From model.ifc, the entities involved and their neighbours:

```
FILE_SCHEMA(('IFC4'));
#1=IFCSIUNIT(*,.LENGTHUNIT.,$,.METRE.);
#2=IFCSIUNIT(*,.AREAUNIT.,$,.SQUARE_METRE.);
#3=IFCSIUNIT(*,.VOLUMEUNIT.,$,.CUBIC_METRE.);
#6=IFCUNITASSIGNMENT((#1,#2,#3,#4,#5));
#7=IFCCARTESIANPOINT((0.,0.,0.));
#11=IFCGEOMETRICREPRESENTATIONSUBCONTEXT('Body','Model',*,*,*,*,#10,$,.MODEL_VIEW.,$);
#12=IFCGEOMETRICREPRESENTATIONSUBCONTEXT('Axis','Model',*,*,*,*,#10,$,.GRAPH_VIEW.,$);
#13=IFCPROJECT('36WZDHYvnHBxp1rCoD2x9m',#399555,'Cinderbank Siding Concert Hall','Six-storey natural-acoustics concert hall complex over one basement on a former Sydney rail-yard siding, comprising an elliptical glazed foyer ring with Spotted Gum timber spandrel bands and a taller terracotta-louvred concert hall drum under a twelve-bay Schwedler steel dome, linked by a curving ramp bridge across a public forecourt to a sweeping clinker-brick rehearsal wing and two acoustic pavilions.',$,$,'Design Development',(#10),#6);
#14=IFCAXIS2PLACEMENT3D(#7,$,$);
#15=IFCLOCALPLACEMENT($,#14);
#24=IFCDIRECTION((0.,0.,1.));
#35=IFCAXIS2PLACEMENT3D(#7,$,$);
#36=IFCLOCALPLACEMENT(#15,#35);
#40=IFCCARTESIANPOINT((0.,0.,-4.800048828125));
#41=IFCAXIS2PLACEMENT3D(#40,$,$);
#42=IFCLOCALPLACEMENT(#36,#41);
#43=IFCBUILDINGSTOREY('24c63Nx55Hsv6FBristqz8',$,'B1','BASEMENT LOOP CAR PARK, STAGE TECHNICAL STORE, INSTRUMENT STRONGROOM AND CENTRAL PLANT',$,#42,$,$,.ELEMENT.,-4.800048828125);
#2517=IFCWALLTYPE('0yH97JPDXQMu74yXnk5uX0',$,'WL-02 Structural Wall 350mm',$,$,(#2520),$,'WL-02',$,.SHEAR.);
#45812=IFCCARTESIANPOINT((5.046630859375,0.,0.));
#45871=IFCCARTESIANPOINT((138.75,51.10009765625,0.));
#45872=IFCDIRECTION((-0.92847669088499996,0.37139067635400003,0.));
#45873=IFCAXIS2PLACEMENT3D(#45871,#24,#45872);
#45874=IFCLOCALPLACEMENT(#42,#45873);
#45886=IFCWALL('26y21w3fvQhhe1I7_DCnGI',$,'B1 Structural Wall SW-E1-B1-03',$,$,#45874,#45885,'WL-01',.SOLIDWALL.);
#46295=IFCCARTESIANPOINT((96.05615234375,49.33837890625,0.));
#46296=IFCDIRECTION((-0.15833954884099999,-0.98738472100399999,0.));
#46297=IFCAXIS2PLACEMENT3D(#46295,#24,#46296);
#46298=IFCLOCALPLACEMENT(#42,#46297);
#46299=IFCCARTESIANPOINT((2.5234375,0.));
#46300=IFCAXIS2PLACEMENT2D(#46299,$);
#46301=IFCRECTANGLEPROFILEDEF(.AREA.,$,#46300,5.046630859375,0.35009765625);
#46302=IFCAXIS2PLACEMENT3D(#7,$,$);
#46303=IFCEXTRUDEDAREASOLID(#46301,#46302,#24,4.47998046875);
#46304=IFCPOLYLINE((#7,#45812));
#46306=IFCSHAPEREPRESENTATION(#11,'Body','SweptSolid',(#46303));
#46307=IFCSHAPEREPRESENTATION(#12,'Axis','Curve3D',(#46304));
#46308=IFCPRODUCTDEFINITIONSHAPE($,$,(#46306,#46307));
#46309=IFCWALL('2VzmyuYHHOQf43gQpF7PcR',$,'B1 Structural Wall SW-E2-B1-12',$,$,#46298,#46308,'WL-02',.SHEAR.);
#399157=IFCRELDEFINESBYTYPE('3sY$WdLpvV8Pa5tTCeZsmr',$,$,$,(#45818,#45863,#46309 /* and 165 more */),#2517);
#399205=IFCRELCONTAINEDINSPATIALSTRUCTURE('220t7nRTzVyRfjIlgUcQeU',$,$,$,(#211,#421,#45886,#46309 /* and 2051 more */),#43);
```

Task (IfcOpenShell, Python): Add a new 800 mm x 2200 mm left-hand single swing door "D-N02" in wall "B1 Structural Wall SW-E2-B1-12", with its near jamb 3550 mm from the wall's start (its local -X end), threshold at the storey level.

```python
import numpy as np
import ifcopenshell
import ifcopenshell.api.feature
import ifcopenshell.api.geometry
import ifcopenshell.api.root
import ifcopenshell.api.spatial
import ifcopenshell.geom
import ifcopenshell.util.element
import ifcopenshell.util.placement
import ifcopenshell.util.representation
import ifcopenshell.util.shape
import ifcopenshell.util.unit

model = ifcopenshell.open("model.ifc")
unit_scale = ifcopenshell.util.unit.calculate_unit_scale(model)
settings = ifcopenshell.geom.settings()


def volume(element):
    """Net volume in cubic metres, openings subtracted."""
    shape = ifcopenshell.geom.create_shape(settings, element)
    return ifcopenshell.util.shape.get_volume(shape.geometry)


wall = model.by_guid("2VzmyuYHHOQf43gQpF7PcR")
storey = ifcopenshell.util.element.get_container(wall, ifc_class="IfcBuildingStorey")
context = ifcopenshell.util.representation.get_context(model, "Model", "Body", "MODEL_VIEW")
before = volume(wall)

width, height, from_end, sill = 0.8, 2.2, 3.55, 0.0  # metres

# The wall runs along its own X axis, and the end named is its -X end.
wall_shape = ifcopenshell.geom.create_shape(settings, wall)
x, y, z = ifcopenshell.util.shape.get_vertices(wall_shape.geometry).T
start = x.min() + from_end
face, thickness = float(y.min()), float(y.max() - y.min())
wall_matrix = ifcopenshell.util.placement.get_local_placement(wall.ObjectPlacement)
level = ifcopenshell.util.placement.get_local_placement(storey.ObjectPlacement)[2, 3]


def in_wall(x, y):
    """Placement at x, y metres in the wall's axes, at sill height."""
    matrix = wall_matrix.copy()
    matrix[:, 3] = wall_matrix @ np.array([x / unit_scale, y / unit_scale, 0.0, 1.0])
    matrix[2, 3] = level + sill / unit_scale
    return matrix


# Opening: a box that overshoots both wall faces by 50 mm.
opening = ifcopenshell.api.root.create_entity(model, ifc_class="IfcOpeningElement", predefined_type="OPENING")
box = ifcopenshell.api.geometry.add_wall_representation(
    model, context=context, length=width, height=height, thickness=thickness + 0.1
)
ifcopenshell.api.geometry.assign_representation(model, product=opening, representation=box)
ifcopenshell.api.geometry.edit_object_placement(model, product=opening, matrix=in_wall(start, face - 0.05), is_si=False)
ifcopenshell.api.feature.add_feature(model, feature=opening, element=wall)

door = ifcopenshell.api.root.create_entity(model, ifc_class="IfcDoor", name="D-N02", predefined_type="DOOR")
door.OverallWidth, door.OverallHeight = width / unit_scale, height / unit_scale
door.OperationType = "SINGLE_SWING_LEFT"
body = ifcopenshell.api.geometry.add_door_representation(
    model,
    context=context,
    overall_width=door.OverallWidth,
    overall_height=door.OverallHeight,
    operation_type="SINGLE_SWING_LEFT",
    lining_properties={"LiningDepth": thickness / unit_scale, "ThresholdDepth": thickness / unit_scale},
)
ifcopenshell.api.geometry.assign_representation(model, product=door, representation=body)
ifcopenshell.api.spatial.assign_container(model, products=[door], relating_structure=storey)
ifcopenshell.api.feature.add_filling(model, opening=opening, element=door)

# The lining spans the wall, so the door starts at the wall face.
ifcopenshell.api.geometry.edit_object_placement(model, product=door, matrix=in_wall(start, face), is_si=False)

after = volume(wall)

print(f"wall volume {before:.3f} -> {after:.3f} m3")

model.write("model_edited.ifc")
```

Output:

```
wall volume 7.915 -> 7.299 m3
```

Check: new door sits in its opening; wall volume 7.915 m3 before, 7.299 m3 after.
